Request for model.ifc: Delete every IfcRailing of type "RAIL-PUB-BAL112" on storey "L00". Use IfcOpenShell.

First a look at what the model holds.

```python
import ifcopenshell
import ifcopenshell.util.element

model = ifcopenshell.open("model.ifc")
print(model.schema)
storey = next(s for s in model.by_type("IfcBuildingStorey") if s.Name == "L00")
railings = [e for e in ifcopenshell.util.element.get_decomposition(storey) if e.is_a("IfcRailing")]
seen = {}
for e in railings:
    element_type = ifcopenshell.util.element.get_type(e)
    name = element_type.Name if element_type not in (None, e) else None
    seen[name] = seen.get(name, 0) + 1
for name, count in sorted(seen.items(), key=str):
    print(count, "x", name)
```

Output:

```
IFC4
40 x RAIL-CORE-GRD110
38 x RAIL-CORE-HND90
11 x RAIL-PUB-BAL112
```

```python
import ifcopenshell
import ifcopenshell.api.root
import ifcopenshell.util.element

model = ifcopenshell.open("model.ifc")

storey = next(s for s in model.by_type("IfcBuildingStorey") if s.Name == "L00")
railings = [e for e in ifcopenshell.util.element.get_decomposition(storey) if e.is_a("IfcRailing")]
targets = [e for e in railings if (t := ifcopenshell.util.element.get_type(e)) not in (None, e) and t.Name == "RAIL-PUB-BAL112"]

for e in targets:
    ifcopenshell.api.root.remove_product(model, product=e)
print(len(targets), "removed")

model.write("model_rev.ifc")
```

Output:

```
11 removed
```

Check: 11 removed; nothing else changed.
